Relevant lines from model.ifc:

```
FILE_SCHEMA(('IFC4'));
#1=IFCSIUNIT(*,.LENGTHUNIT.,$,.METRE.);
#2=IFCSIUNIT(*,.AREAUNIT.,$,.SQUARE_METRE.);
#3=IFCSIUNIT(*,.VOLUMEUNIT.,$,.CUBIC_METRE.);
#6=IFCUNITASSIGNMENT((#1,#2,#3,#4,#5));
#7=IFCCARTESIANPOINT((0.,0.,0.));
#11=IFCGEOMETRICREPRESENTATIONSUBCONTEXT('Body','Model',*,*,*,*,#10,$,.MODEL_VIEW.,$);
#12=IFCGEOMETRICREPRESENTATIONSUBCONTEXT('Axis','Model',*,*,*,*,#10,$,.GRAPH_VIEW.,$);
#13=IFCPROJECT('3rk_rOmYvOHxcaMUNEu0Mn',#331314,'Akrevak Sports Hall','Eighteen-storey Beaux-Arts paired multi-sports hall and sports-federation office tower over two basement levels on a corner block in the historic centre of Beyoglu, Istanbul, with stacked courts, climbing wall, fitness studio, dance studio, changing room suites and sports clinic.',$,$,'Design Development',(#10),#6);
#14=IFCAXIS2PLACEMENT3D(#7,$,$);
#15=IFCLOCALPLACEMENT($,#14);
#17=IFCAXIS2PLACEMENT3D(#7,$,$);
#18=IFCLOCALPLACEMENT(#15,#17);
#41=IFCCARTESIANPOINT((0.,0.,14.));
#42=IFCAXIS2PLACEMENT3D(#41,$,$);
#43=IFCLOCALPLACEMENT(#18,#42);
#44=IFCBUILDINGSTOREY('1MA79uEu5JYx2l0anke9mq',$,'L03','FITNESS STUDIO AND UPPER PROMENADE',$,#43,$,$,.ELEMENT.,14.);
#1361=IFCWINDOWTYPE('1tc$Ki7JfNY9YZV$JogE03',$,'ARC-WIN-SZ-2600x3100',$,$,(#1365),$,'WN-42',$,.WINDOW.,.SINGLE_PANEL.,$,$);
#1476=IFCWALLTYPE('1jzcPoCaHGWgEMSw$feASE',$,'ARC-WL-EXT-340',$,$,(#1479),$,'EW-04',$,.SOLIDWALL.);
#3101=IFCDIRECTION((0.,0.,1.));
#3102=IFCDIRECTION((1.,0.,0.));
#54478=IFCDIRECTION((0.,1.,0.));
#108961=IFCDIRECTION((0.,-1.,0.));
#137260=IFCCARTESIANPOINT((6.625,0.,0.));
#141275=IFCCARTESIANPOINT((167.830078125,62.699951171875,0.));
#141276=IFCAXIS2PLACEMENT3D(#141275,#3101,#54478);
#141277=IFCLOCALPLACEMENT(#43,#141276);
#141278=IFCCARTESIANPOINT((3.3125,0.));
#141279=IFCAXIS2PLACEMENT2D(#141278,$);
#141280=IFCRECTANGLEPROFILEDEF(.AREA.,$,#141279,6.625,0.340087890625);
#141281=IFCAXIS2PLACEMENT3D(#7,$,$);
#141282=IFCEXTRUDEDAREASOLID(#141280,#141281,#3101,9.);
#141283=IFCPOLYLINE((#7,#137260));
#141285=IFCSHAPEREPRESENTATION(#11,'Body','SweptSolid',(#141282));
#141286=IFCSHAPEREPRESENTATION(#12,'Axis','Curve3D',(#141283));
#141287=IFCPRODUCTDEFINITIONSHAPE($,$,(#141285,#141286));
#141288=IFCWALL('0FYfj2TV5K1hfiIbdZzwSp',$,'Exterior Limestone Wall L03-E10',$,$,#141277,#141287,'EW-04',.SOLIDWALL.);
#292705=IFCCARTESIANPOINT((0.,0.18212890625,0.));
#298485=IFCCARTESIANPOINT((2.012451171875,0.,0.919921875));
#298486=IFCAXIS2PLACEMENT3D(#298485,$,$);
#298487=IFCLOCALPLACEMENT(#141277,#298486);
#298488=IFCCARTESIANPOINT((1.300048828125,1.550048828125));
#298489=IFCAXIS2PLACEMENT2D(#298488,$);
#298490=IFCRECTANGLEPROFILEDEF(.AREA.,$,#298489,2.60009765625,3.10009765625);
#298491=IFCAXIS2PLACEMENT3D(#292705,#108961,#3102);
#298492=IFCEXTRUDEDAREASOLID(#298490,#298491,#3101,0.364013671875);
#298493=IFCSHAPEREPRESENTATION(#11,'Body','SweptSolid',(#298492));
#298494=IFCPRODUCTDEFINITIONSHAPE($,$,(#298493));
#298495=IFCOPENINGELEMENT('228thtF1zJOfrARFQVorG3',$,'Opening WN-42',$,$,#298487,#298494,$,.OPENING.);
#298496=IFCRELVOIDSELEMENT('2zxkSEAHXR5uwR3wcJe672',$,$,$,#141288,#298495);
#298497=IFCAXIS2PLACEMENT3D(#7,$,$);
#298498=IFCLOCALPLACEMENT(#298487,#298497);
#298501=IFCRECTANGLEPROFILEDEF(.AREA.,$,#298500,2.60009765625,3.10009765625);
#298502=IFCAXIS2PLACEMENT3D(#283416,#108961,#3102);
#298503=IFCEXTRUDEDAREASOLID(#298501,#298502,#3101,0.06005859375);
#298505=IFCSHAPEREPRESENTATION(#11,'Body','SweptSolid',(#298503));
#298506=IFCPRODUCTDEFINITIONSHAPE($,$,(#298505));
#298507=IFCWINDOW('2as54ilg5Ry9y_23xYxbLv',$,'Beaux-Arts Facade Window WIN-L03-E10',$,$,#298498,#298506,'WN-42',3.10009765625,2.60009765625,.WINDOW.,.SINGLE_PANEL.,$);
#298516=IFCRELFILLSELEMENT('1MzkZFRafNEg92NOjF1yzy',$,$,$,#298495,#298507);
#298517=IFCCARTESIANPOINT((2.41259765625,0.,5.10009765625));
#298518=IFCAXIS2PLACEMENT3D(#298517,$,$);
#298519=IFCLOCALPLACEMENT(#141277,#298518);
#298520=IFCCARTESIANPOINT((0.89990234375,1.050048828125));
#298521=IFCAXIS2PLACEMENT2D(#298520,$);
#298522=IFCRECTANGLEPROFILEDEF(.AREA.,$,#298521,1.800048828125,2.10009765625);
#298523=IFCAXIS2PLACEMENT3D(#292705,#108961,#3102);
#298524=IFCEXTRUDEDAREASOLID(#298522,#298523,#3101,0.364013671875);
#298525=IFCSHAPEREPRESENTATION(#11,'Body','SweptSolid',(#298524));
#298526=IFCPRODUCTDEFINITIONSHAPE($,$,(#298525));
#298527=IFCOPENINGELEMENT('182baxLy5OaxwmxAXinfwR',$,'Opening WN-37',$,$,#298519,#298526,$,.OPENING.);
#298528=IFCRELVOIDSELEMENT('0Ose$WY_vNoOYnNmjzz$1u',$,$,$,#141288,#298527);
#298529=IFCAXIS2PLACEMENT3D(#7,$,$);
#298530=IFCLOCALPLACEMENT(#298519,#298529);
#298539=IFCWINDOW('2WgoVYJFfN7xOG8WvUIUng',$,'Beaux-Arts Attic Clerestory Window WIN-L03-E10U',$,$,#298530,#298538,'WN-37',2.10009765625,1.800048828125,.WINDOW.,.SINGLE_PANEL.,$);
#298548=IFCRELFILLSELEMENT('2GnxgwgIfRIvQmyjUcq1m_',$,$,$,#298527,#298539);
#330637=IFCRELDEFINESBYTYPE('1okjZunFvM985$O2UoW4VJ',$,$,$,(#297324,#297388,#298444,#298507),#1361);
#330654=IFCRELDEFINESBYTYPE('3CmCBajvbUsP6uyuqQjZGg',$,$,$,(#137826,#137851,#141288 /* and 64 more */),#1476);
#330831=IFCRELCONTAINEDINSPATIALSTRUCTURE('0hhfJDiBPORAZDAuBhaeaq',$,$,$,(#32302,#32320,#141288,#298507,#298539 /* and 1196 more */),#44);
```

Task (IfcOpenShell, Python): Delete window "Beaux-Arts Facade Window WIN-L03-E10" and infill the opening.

```python
import ifcopenshell
import ifcopenshell.api.feature
import ifcopenshell.api.root
import ifcopenshell.geom
import ifcopenshell.util.shape

model = ifcopenshell.open("model.ifc")
settings = ifcopenshell.geom.settings()


def volume(element):
    """Net volume in cubic metres, openings subtracted."""
    shape = ifcopenshell.geom.create_shape(settings, element)
    return ifcopenshell.util.shape.get_volume(shape.geometry)


window = model.by_id(298507)
opening = window.FillsVoids[0].RelatingOpeningElement
wall = opening.VoidsElements[0].RelatingBuildingElement
before = volume(wall)

ifcopenshell.api.root.remove_product(model, product=window)
ifcopenshell.api.feature.remove_feature(model, feature=opening)

after = volume(wall)

print(f"wall volume {before:.3f} -> {after:.3f} m3")

model.write("model_edited.ifc")
```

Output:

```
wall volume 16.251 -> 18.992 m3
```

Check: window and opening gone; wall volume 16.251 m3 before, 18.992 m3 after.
